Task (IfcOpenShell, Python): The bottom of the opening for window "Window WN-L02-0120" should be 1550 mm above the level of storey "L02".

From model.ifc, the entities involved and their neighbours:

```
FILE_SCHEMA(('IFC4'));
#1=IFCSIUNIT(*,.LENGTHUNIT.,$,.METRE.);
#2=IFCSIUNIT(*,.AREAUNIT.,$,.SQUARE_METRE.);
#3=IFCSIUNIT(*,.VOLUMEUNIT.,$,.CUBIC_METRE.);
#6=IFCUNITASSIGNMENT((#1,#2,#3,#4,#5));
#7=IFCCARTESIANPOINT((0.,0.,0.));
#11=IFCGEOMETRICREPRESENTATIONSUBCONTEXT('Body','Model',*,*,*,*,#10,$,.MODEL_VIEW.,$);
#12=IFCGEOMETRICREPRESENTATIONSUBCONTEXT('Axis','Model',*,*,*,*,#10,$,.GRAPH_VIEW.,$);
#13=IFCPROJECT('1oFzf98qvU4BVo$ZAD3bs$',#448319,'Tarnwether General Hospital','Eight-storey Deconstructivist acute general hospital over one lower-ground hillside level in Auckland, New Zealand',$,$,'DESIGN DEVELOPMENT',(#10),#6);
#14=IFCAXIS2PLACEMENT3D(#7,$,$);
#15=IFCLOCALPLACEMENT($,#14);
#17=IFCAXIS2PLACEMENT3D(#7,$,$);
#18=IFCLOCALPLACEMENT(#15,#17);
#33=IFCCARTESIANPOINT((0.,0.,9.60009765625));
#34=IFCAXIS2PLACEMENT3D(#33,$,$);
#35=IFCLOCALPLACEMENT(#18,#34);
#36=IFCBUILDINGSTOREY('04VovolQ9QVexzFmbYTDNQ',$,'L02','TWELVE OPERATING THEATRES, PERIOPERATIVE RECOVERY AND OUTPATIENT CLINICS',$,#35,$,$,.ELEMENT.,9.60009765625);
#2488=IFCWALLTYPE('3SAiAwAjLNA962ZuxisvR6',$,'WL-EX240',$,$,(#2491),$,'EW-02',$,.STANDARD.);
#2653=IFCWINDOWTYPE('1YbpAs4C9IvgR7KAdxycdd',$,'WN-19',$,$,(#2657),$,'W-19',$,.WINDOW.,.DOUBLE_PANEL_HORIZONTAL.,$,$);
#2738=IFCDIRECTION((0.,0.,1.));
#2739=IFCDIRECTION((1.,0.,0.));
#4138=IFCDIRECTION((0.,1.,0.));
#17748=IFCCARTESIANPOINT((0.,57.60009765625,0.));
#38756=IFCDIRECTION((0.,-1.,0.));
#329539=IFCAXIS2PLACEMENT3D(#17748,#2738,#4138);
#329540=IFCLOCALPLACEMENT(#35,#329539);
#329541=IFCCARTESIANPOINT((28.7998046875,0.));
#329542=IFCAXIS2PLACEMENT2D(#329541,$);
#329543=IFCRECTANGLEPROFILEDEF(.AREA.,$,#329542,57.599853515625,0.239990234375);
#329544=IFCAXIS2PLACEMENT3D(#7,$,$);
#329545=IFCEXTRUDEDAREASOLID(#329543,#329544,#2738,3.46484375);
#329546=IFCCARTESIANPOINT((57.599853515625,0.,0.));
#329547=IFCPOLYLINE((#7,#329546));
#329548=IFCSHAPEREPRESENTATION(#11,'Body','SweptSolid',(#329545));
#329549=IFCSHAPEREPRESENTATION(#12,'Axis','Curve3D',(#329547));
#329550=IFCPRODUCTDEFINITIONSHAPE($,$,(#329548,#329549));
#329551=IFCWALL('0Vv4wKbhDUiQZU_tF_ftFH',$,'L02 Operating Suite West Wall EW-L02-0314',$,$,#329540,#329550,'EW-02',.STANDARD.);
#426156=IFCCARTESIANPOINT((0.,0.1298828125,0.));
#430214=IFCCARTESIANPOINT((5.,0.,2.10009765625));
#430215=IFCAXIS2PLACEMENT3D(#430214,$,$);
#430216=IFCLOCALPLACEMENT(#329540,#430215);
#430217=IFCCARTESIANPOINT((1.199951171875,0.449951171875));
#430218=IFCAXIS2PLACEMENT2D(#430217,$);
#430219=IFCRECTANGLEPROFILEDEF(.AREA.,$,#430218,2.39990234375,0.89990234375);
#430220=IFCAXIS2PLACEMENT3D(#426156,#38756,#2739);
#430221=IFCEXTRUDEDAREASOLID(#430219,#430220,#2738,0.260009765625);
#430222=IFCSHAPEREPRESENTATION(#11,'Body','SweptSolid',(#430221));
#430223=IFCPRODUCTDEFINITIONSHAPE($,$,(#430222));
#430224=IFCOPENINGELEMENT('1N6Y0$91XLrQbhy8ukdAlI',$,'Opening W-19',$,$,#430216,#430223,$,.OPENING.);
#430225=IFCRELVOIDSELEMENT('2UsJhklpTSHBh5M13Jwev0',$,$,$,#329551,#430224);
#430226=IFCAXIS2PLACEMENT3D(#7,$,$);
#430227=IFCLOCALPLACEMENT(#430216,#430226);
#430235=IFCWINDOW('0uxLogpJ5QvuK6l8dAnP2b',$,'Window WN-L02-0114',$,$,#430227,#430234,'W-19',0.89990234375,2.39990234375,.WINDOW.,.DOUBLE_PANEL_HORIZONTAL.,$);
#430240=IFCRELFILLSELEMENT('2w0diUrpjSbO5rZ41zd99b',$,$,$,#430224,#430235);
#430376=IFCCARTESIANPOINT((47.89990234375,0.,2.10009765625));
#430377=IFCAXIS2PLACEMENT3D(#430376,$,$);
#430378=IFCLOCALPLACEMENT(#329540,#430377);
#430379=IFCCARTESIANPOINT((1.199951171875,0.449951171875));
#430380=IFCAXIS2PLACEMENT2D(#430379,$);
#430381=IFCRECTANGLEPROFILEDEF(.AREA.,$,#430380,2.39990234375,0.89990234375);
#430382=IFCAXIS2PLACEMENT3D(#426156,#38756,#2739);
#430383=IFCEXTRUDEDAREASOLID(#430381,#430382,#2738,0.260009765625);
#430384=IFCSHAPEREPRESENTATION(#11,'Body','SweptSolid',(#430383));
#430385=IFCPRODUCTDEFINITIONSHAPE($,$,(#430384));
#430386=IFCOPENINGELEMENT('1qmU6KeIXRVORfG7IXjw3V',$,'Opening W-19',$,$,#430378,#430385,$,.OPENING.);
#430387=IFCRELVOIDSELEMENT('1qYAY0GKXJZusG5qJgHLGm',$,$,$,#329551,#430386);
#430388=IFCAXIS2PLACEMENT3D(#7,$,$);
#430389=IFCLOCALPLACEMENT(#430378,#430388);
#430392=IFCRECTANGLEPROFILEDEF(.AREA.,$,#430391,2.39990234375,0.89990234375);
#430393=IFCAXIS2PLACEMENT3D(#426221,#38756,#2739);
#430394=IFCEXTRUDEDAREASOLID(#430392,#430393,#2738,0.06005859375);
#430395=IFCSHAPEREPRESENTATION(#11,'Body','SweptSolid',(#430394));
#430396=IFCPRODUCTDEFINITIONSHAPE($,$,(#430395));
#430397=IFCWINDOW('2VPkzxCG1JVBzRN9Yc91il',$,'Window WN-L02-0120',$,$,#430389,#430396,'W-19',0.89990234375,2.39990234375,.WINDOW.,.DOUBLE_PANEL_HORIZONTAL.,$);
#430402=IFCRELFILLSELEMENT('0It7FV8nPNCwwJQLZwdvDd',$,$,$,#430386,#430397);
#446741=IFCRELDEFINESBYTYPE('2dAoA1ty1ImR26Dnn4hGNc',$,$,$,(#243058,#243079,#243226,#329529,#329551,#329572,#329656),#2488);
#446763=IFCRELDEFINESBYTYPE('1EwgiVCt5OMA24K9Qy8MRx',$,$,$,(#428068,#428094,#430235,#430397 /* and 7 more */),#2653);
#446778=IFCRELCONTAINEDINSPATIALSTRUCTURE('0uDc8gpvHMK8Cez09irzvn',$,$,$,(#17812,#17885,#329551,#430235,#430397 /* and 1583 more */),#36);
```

```python
import numpy as np
import ifcopenshell
import ifcopenshell.api.geometry
import ifcopenshell.geom
import ifcopenshell.util.element
import ifcopenshell.util.placement
import ifcopenshell.util.shape
import ifcopenshell.util.unit

model = ifcopenshell.open("model.ifc")
unit_scale = ifcopenshell.util.unit.calculate_unit_scale(model)

window = model.by_guid("2VPkzxCG1JVBzRN9Yc91il")
opening = window.FillsVoids[0].RelatingOpeningElement
storey = ifcopenshell.util.element.get_container(window, ifc_class="IfcBuildingStorey")
level = ifcopenshell.util.placement.get_local_placement(storey.ObjectPlacement)[2, 3]

# The opening's origin need not be at the sill, so measure its lowest point.
shape = ifcopenshell.geom.create_shape(ifcopenshell.geom.settings(), opening)
bottom = ifcopenshell.util.shape.get_shape_bottom_elevation(shape, shape.geometry) / unit_scale
dz = level + 1.55 / unit_scale - bottom

shift = np.array([0.0, 0.0, dz])
# The window is placed relative to its opening, so it follows when the opening moves.
matrix = ifcopenshell.util.placement.get_local_placement(opening.ObjectPlacement)
matrix[:3, 3] += shift
ifcopenshell.api.geometry.edit_object_placement(
    model, product=opening, matrix=matrix, is_si=False, should_transform_children=True
)

print(f"moved by {dz * unit_scale:+.3f} m")

model.write("model_v2.ifc")
```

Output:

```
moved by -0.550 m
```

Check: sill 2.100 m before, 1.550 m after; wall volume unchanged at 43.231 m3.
